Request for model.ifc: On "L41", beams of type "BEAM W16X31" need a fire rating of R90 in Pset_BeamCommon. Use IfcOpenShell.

First a look at what the model holds.

```python
import ifcopenshell
import ifcopenshell.util.element

model = ifcopenshell.open("model.ifc")
print(model.schema)
storey = next(s for s in model.by_type("IfcBuildingStorey") if s.Name == "L41")
beams = [e for e in ifcopenshell.util.element.get_decomposition(storey) if e.is_a("IfcBeam")]
seen = {}
for e in beams:
    element_type = ifcopenshell.util.element.get_type(e)
    key = (element_type.Name if element_type != e and element_type else None, ifcopenshell.util.element.get_pset(e, "Pset_BeamCommon", "FireRating"))
    seen[key] = seen.get(key, 0) + 1
for (name, value), count in sorted(seen.items(), key=str):
    print(count, "x", name, "|", value)
```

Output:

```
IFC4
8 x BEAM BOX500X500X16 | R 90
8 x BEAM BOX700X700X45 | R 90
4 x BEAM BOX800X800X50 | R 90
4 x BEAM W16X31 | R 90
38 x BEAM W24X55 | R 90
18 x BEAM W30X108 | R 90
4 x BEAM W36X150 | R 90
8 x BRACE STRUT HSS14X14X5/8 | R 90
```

```python
import ifcopenshell
import ifcopenshell.api.pset
import ifcopenshell.util.element

model = ifcopenshell.open("model.ifc")

storey = next(s for s in model.by_type("IfcBuildingStorey") if s.Name == "L41")
beams = [e for e in ifcopenshell.util.element.get_decomposition(storey) if e.is_a("IfcBeam")]

count = 0
for e in beams:
    element_type = ifcopenshell.util.element.get_type(e)
    if element_type in (None, e) or element_type.Name != "BEAM W16X31":
        continue
    found = ifcopenshell.util.element.get_pset(e, "Pset_BeamCommon", should_inherit=False)
    if found:
        pset = model.by_id(found["id"])
        if len(ifcopenshell.util.element.get_elements_by_pset(pset)) > 1:
            pset = ifcopenshell.api.pset.unshare_pset(model, products=[e], pset=pset)[0]
    else:
        pset = ifcopenshell.api.pset.add_pset(model, product=e, name="Pset_BeamCommon")
    ifcopenshell.api.pset.edit_pset(model, pset=pset, properties={"FireRating": "R90"})
    count += 1

print(count, "beams updated")

model.write("model_rev.ifc")
```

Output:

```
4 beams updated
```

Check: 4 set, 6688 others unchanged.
